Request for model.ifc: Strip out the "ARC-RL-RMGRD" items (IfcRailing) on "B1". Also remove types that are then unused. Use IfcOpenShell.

First a look at what the model holds.

```python
import ifcopenshell
import ifcopenshell.util.element

model = ifcopenshell.open("model.ifc")
print(model.schema)
storey = next(s for s in model.by_type("IfcBuildingStorey") if s.Name == "B1")
railings = [e for e in ifcopenshell.util.element.get_decomposition(storey) if e.is_a("IfcRailing")]
seen = {}
for e in railings:
    element_type = ifcopenshell.util.element.get_type(e)
    name = element_type.Name if element_type not in (None, e) else None
    seen[name] = seen.get(name, 0) + 1
for name, count in sorted(seen.items(), key=str):
    print(count, "x", name)
```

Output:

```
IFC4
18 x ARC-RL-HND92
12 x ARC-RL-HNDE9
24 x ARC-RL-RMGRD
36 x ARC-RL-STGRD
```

```python
import ifcopenshell
import ifcopenshell.api.root
import ifcopenshell.util.element

model = ifcopenshell.open("model.ifc")

storey = next(s for s in model.by_type("IfcBuildingStorey") if s.Name == "B1")
railings = [e for e in ifcopenshell.util.element.get_decomposition(storey) if e.is_a("IfcRailing")]
targets = [e for e in railings if (t := ifcopenshell.util.element.get_type(e)) not in (None, e) and t.Name == "ARC-RL-RMGRD"]
types = {ifcopenshell.util.element.get_type(e) for e in targets} - {None, *targets}

for e in targets:
    ifcopenshell.api.root.remove_product(model, product=e)
print(len(targets), "removed")

unused = [t for t in types if not ifcopenshell.util.element.get_types(t)]
for t in unused:
    ifcopenshell.api.root.remove_product(model, product=t)
print(len(unused), "unused types removed")

model.write("model_updated.ifc")
```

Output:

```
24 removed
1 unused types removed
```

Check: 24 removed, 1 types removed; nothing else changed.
